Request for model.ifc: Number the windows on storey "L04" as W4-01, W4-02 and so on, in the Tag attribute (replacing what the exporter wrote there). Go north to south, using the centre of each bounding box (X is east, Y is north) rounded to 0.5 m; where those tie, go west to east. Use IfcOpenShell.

First a look at what the model holds.

```python
import ifcopenshell
import ifcopenshell.util.element
import ifcopenshell.util.placement

model = ifcopenshell.open("model.ifc")
print(model.schema)
storey = next(s for s in model.by_type("IfcBuildingStorey") if s.Name == "L04")
windows = [e for e in ifcopenshell.util.element.get_decomposition(storey) if e.is_a("IfcWindow")]
for e in sorted(windows, key=lambda e: e.id()):
    origin = ifcopenshell.util.placement.get_local_placement(e.ObjectPlacement)[:3, 3]
    print(e.id(), e.Tag, e.Name, origin.round(2) + 0.0, sep=" | ")
```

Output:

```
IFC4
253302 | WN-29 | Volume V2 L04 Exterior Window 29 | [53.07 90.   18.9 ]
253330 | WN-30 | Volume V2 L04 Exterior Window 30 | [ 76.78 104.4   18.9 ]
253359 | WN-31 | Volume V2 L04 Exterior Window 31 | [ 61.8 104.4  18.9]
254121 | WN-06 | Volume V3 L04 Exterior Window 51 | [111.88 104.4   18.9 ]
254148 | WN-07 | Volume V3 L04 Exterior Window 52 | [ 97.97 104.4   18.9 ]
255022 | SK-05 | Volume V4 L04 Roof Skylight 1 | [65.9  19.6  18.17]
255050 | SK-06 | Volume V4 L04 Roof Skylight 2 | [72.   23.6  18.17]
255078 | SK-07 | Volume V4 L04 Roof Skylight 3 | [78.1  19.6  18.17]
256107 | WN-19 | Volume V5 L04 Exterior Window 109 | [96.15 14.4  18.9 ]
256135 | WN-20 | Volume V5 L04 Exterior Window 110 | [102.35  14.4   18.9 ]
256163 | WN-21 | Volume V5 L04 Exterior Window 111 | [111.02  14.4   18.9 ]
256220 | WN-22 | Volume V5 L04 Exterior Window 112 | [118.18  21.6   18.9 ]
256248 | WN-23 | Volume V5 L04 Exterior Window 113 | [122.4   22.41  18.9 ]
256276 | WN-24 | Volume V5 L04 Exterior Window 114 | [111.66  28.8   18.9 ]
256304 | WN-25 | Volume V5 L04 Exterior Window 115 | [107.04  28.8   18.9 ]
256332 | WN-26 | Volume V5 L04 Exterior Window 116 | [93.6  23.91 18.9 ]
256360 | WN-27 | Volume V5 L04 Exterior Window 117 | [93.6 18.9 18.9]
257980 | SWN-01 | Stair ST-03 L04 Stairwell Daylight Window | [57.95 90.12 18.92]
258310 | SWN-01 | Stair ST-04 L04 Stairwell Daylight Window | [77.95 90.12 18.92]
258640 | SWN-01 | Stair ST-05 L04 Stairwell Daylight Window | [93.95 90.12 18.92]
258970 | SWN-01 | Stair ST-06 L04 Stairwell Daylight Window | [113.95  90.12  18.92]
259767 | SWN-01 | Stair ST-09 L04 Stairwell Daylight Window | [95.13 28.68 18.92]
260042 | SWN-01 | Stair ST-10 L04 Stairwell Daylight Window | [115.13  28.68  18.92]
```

```python
import ifcopenshell
import ifcopenshell.geom
import ifcopenshell.util.element
import ifcopenshell.util.shape

model = ifcopenshell.open("model.ifc")
settings = ifcopenshell.geom.settings()
settings.set("use-world-coords", True)


def centre(element):
    shape = ifcopenshell.geom.create_shape(settings, element)
    return ifcopenshell.util.shape.get_bbox_centroid(shape.geometry)


storey = next(s for s in model.by_type("IfcBuildingStorey") if s.Name == "L04")
windows = [e for e in ifcopenshell.util.element.get_decomposition(storey) if e.is_a("IfcWindow")]

# Insertion points can sit at a corner or the storey origin, so sort by the geometry (in metres).
centres = {e: centre(e) for e in windows}
windows.sort(key=lambda e: (-round(centres[e][1] / 0.5), centres[e][0]))

for i, e in enumerate(windows, start=1):
    number = f"W4-{i:02d}"
    e.Tag = number
    print(e.id(), number)

model.write("model_v2.ifc")
```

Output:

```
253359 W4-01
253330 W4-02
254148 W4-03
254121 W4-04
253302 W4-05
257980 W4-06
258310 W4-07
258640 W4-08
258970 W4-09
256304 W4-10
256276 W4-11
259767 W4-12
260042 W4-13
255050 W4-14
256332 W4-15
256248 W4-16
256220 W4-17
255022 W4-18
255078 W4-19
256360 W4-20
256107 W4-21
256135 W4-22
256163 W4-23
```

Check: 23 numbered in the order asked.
